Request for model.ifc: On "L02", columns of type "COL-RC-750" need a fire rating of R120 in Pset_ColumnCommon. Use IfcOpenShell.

First a look at what the model holds.

```python
import ifcopenshell
import ifcopenshell.util.element

model = ifcopenshell.open("model.ifc")
print(model.schema)
storey = next(s for s in model.by_type("IfcBuildingStorey") if s.Name == "L02")
columns = [e for e in ifcopenshell.util.element.get_decomposition(storey) if e.is_a("IfcColumn")]
seen = {}
for e in columns:
    element_type = ifcopenshell.util.element.get_type(e)
    key = (element_type.Name if element_type != e and element_type else None, ifcopenshell.util.element.get_pset(e, "Pset_ColumnCommon", "FireRating"))
    seen[key] = seen.get(key, 0) + 1
for (name, value), count in sorted(seen.items(), key=str):
    print(count, "x", name, "|", value)
```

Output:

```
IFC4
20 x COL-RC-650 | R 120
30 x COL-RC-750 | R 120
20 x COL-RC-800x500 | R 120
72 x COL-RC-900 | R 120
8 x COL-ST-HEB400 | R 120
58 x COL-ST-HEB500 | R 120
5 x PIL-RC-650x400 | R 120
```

```python
import ifcopenshell
import ifcopenshell.api.pset
import ifcopenshell.util.element

model = ifcopenshell.open("model.ifc")

storey = next(s for s in model.by_type("IfcBuildingStorey") if s.Name == "L02")
columns = [e for e in ifcopenshell.util.element.get_decomposition(storey) if e.is_a("IfcColumn")]

count = 0
for e in columns:
    element_type = ifcopenshell.util.element.get_type(e)
    if element_type in (None, e) or element_type.Name != "COL-RC-750":
        continue
    # add_pset returns the element's existing set when there is one.
    pset = ifcopenshell.api.pset.add_pset(model, product=e, name="Pset_ColumnCommon")
    ifcopenshell.api.pset.edit_pset(model, pset=pset, properties={"FireRating": "R120"})
    count += 1

print(count, "columns updated")

model.write("model_edited.ifc")
```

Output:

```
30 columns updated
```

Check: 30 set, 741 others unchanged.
